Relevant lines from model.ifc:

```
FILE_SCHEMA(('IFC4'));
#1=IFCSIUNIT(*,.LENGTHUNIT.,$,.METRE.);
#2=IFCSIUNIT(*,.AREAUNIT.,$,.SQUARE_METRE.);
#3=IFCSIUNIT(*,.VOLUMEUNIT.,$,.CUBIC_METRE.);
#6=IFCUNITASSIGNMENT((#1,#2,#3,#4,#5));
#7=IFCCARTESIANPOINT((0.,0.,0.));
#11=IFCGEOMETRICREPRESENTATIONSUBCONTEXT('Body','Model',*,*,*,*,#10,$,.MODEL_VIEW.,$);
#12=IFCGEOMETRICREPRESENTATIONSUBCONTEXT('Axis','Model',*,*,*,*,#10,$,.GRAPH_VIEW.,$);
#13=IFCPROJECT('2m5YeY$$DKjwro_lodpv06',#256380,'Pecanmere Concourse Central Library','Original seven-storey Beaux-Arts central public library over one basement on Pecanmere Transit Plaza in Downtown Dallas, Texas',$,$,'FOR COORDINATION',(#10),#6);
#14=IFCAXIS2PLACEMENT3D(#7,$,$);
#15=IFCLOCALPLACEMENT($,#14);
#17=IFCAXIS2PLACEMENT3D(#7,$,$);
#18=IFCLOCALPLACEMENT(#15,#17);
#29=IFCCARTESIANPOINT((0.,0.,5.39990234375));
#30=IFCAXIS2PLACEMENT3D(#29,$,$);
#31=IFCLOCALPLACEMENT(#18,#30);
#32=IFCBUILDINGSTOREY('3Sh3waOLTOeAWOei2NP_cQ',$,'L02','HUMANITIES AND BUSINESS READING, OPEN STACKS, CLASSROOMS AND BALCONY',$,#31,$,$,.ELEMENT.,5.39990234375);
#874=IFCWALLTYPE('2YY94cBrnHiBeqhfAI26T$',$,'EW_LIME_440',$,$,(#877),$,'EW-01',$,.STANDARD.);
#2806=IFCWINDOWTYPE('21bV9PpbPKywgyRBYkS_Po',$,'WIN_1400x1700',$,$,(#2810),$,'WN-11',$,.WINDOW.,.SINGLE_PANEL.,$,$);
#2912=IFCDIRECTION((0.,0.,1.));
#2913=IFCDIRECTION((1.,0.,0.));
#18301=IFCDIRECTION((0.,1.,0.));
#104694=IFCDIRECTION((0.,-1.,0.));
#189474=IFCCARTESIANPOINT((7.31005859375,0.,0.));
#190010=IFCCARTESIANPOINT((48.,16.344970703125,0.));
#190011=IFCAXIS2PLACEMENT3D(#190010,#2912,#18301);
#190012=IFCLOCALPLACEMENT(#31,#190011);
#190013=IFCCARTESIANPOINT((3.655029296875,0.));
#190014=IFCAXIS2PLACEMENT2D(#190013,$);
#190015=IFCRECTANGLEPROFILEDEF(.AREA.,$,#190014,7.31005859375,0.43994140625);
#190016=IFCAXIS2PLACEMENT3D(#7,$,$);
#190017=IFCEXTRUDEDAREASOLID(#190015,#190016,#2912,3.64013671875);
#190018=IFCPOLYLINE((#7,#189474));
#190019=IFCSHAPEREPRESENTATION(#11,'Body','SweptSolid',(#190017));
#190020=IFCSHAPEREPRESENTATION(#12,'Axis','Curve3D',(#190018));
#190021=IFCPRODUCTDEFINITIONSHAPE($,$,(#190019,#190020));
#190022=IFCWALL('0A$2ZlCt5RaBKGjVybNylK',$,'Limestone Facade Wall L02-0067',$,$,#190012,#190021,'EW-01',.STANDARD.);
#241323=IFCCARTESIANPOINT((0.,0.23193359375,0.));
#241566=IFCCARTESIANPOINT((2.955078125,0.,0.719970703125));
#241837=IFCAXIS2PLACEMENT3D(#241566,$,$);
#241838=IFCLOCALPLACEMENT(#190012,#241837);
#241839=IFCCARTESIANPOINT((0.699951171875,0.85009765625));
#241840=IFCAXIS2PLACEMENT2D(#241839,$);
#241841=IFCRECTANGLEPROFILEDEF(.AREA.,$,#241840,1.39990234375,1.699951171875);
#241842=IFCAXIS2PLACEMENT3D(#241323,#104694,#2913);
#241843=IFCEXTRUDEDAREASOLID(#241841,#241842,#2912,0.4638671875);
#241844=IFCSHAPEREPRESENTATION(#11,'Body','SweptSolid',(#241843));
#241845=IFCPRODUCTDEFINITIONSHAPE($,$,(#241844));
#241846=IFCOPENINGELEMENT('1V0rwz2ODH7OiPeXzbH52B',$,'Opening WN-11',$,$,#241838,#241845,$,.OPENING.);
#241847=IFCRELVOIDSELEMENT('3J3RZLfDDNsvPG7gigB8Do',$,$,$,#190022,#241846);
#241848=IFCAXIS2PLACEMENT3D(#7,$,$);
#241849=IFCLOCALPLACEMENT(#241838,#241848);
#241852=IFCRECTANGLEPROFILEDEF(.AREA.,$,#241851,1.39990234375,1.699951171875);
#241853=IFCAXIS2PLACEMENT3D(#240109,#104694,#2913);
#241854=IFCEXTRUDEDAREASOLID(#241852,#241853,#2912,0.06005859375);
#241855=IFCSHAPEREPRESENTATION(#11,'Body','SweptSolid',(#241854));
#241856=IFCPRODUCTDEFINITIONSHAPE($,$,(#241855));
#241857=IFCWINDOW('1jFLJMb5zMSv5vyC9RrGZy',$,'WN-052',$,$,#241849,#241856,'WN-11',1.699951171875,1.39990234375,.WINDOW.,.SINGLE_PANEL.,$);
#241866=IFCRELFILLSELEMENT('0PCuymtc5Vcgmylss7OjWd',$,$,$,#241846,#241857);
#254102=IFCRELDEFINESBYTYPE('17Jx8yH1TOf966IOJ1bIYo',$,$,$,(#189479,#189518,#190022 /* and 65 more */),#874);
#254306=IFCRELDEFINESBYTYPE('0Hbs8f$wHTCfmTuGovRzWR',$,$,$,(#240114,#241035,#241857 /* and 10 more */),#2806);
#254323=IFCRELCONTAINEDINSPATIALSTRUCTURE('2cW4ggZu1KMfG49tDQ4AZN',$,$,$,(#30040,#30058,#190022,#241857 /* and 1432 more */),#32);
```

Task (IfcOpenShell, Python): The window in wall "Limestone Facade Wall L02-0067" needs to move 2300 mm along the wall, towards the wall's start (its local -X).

```python
import ifcopenshell
import ifcopenshell.api.geometry
import ifcopenshell.util.placement
import ifcopenshell.util.unit

model = ifcopenshell.open("model.ifc")
unit_scale = ifcopenshell.util.unit.calculate_unit_scale(model)

window = model.by_guid("1jFLJMb5zMSv5vyC9RrGZy")
opening = window.FillsVoids[0].RelatingOpeningElement
wall = opening.VoidsElements[0].RelatingBuildingElement

wall_matrix = ifcopenshell.util.placement.get_local_placement(wall.ObjectPlacement)
shift = wall_matrix[:3, 0] * -2.3 / unit_scale
before = ifcopenshell.util.placement.get_local_placement(window.ObjectPlacement)[:3, 3].copy()

# The window is placed relative to its opening, so it follows when the opening moves.
matrix = ifcopenshell.util.placement.get_local_placement(opening.ObjectPlacement)
matrix[:3, 3] += shift
ifcopenshell.api.geometry.edit_object_placement(
    model, product=opening, matrix=matrix, is_si=False, should_transform_children=True
)

after = ifcopenshell.util.placement.get_local_placement(window.ObjectPlacement)[:3, 3]
print("window moved by", (after - before).round(3) + 0.0)

model.write("model_updated.ifc")
```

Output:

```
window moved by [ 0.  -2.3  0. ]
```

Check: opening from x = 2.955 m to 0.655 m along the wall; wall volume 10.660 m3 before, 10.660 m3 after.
